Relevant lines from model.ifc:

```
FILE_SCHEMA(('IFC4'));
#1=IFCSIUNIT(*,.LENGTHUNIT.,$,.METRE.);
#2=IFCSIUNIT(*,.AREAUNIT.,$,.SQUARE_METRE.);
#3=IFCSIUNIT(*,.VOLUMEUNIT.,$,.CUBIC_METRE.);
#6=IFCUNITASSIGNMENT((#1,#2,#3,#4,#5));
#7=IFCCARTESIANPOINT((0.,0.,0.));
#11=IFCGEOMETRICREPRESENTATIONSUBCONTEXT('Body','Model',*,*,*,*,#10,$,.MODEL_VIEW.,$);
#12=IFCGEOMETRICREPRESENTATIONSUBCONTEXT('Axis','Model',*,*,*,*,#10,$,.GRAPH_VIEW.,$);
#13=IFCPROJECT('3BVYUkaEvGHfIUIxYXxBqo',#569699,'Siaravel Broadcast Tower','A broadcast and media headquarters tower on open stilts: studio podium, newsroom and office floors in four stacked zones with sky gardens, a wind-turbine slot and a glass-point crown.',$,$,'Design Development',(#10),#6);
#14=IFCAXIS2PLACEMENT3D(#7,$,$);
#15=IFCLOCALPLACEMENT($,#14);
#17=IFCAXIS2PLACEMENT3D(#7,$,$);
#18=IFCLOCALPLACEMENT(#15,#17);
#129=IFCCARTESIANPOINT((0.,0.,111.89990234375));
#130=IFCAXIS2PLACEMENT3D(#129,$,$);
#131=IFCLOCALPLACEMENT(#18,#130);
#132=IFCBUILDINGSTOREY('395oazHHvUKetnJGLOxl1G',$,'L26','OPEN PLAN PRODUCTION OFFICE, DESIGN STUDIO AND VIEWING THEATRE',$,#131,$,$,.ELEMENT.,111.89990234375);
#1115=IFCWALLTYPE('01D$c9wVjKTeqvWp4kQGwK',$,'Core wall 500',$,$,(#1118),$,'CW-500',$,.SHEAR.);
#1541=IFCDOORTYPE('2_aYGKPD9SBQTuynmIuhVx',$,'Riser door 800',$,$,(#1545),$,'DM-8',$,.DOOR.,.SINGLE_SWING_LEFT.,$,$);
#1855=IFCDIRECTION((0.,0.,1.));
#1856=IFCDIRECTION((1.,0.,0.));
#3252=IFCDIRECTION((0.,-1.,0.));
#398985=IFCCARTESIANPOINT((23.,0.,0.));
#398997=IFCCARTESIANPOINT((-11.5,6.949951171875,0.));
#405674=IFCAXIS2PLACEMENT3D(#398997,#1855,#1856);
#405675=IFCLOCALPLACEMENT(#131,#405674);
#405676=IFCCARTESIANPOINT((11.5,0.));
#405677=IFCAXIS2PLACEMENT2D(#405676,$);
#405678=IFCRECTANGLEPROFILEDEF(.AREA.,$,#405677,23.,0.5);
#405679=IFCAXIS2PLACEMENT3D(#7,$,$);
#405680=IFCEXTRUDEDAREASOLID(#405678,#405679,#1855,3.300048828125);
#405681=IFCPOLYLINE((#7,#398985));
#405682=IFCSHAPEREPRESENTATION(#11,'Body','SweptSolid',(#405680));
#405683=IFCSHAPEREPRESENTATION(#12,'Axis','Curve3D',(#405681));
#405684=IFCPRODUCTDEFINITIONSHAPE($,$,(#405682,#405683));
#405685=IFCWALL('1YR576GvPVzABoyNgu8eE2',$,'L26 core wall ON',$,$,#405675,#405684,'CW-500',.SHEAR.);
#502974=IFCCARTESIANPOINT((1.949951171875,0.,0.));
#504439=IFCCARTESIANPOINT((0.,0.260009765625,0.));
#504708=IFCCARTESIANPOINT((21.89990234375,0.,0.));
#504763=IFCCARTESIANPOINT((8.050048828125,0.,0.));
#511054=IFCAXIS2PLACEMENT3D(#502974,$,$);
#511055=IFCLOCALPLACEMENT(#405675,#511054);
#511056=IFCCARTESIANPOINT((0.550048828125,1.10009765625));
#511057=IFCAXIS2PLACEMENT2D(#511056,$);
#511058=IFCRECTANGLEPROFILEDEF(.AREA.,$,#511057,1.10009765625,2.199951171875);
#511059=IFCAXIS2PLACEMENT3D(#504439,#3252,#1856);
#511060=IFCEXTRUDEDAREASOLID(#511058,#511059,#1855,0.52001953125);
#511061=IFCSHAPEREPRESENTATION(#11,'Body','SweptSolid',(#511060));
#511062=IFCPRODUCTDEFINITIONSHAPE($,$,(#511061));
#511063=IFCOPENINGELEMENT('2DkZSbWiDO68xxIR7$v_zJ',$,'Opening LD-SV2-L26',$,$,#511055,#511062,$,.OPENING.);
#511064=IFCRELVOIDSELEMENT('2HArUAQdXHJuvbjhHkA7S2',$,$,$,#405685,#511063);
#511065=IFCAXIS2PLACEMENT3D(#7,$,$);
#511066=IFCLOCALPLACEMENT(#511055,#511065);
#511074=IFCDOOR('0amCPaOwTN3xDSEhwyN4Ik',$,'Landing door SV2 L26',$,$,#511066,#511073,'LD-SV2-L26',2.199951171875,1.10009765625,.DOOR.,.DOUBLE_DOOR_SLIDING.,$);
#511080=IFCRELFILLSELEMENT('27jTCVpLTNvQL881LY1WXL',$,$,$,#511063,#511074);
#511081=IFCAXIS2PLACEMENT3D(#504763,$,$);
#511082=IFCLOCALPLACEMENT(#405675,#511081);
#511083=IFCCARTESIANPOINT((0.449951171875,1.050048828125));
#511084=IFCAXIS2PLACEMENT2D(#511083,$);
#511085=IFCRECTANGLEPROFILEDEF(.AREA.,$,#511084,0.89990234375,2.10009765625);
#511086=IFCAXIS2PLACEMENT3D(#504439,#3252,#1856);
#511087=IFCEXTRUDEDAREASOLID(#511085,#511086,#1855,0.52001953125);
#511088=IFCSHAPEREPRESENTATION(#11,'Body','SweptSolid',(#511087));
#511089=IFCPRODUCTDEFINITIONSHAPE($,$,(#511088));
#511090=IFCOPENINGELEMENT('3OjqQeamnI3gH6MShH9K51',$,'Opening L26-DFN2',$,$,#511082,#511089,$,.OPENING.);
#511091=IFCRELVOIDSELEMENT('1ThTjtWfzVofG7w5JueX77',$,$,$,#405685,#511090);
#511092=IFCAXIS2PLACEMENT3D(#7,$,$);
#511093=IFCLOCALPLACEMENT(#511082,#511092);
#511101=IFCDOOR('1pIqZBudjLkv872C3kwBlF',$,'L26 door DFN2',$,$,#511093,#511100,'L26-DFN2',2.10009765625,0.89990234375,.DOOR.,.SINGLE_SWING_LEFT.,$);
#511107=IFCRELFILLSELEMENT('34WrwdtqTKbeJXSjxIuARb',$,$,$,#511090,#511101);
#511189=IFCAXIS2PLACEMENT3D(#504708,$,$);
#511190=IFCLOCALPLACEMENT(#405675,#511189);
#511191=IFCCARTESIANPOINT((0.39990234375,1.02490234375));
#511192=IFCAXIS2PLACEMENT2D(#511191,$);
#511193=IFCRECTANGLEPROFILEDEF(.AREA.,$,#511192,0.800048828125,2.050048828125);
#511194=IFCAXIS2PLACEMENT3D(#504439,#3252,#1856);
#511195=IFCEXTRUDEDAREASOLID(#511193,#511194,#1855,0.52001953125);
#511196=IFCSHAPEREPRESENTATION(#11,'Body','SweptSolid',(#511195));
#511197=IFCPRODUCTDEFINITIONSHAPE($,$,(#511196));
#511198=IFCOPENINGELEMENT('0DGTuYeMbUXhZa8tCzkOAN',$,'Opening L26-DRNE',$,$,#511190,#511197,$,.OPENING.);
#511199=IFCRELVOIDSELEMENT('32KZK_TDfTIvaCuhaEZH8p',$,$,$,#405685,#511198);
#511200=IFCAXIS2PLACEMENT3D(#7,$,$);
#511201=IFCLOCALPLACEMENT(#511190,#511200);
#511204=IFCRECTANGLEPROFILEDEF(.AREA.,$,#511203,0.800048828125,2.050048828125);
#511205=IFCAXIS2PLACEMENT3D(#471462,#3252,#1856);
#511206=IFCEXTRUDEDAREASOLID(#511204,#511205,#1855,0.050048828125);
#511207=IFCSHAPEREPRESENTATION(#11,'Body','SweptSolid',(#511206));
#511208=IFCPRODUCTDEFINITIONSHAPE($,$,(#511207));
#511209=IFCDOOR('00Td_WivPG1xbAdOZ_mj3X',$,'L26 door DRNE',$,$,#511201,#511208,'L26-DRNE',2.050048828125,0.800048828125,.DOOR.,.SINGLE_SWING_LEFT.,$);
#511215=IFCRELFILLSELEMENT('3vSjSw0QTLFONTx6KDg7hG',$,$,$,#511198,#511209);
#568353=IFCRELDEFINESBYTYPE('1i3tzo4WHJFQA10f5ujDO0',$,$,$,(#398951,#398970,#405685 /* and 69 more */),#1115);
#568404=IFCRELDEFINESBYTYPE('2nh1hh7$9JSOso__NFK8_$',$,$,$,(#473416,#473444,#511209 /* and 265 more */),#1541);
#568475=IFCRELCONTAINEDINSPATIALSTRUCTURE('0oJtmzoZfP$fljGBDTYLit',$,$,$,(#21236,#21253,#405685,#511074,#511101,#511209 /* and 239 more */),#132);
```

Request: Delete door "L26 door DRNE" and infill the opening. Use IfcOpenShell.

```python
import ifcopenshell
import ifcopenshell.api.feature
import ifcopenshell.api.root
import ifcopenshell.geom
import ifcopenshell.util.shape

model = ifcopenshell.open("model.ifc")
settings = ifcopenshell.geom.settings()


def volume(element):
    """Net volume in cubic metres, openings subtracted."""
    shape = ifcopenshell.geom.create_shape(settings, element)
    return ifcopenshell.util.shape.get_volume(shape.geometry)


door = model.by_guid("00Td_WivPG1xbAdOZ_mj3X")
opening = door.FillsVoids[0].RelatingOpeningElement
wall = opening.VoidsElements[0].RelatingBuildingElement
before = volume(wall)

ifcopenshell.api.root.remove_product(model, product=door)
ifcopenshell.api.feature.remove_feature(model, feature=opening)

after = volume(wall)

print(f"wall volume {before:.3f} -> {after:.3f} m3")

model.write("model_edited.ifc")
```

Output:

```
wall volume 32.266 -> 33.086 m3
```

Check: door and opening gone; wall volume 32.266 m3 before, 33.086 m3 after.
